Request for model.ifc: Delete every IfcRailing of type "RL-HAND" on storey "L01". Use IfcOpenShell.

First a look at what the model holds.

```python
import ifcopenshell
import ifcopenshell.util.element

model = ifcopenshell.open("model.ifc")
print(model.schema)
storey = next(s for s in model.by_type("IfcBuildingStorey") if s.Name == "L01")
railings = [e for e in ifcopenshell.util.element.get_decomposition(storey) if e.is_a("IfcRailing")]
seen = {}
for e in railings:
    element_type = ifcopenshell.util.element.get_type(e)
    name = element_type.Name if element_type not in (None, e) else None
    seen[name] = seen.get(name, 0) + 1
for name, count in sorted(seen.items(), key=str):
    print(count, "x", name)
```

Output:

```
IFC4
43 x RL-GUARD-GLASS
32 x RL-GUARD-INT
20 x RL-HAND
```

```python
import ifcopenshell
import ifcopenshell.api.root
import ifcopenshell.util.element

model = ifcopenshell.open("model.ifc")

storey = next(s for s in model.by_type("IfcBuildingStorey") if s.Name == "L01")
railings = [e for e in ifcopenshell.util.element.get_decomposition(storey) if e.is_a("IfcRailing")]
targets = [e for e in railings if (t := ifcopenshell.util.element.get_type(e)) not in (None, e) and t.Name == "RL-HAND"]

for e in targets:
    ifcopenshell.api.root.remove_product(model, product=e)
print(len(targets), "removed")

model.write("model_v2.ifc")
```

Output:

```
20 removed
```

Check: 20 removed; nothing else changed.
